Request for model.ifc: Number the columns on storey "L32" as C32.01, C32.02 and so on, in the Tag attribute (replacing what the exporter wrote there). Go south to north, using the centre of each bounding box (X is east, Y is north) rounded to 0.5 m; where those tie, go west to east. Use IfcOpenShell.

First a look at what the model holds.

```python
import ifcopenshell
import ifcopenshell.util.element
import ifcopenshell.util.placement

model = ifcopenshell.open("model.ifc")
print(model.schema)
storey = next(s for s in model.by_type("IfcBuildingStorey") if s.Name == "L32")
columns = [e for e in ifcopenshell.util.element.get_decomposition(storey) if e.is_a("IfcColumn")]
for e in sorted(columns, key=lambda e: e.id()):
    origin = ifcopenshell.util.placement.get_local_placement(e.ObjectPlacement)[:3, 3]
    print(e.id(), e.Tag, e.Name, origin.round(2) + 0.0, sep=" | ")
```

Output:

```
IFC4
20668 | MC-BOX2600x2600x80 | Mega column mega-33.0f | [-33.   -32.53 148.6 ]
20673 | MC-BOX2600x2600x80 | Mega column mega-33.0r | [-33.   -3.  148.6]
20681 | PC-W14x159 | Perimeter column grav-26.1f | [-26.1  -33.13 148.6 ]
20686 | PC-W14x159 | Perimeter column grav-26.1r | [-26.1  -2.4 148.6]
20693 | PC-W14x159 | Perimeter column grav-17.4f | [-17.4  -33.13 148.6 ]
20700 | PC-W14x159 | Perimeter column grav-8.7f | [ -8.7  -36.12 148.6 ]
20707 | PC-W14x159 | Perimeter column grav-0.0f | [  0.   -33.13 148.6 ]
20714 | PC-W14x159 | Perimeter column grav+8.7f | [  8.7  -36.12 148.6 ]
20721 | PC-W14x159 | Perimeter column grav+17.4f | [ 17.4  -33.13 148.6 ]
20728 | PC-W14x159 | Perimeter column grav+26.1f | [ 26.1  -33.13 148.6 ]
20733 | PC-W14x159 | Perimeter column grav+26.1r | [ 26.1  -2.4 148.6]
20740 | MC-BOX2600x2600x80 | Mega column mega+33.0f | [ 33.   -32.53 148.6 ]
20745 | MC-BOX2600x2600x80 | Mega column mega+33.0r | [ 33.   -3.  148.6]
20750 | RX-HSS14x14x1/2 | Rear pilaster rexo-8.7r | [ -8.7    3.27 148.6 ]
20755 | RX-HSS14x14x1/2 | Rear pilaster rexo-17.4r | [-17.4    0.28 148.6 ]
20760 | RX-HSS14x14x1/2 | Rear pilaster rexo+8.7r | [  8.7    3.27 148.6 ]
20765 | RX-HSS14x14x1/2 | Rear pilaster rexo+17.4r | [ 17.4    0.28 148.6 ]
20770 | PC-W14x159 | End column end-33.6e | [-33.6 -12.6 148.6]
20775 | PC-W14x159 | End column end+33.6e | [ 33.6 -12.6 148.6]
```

```python
import ifcopenshell
import ifcopenshell.geom
import ifcopenshell.util.element
import ifcopenshell.util.shape

model = ifcopenshell.open("model.ifc")
settings = ifcopenshell.geom.settings()
settings.set("use-world-coords", True)


def centre(element):
    shape = ifcopenshell.geom.create_shape(settings, element)
    return ifcopenshell.util.shape.get_bbox_centroid(shape.geometry)


storey = next(s for s in model.by_type("IfcBuildingStorey") if s.Name == "L32")
columns = [e for e in ifcopenshell.util.element.get_decomposition(storey) if e.is_a("IfcColumn")]

# Insertion points can sit at a corner or the storey origin, so sort by the geometry (in metres).
centres = {e: centre(e) for e in columns}
columns.sort(key=lambda e: (round(centres[e][1] / 0.5), centres[e][0]))

for i, e in enumerate(columns, start=1):
    number = f"C32.{i:02d}"
    e.Tag = number
    print(e.id(), number)

model.write("model_updated.ifc")
```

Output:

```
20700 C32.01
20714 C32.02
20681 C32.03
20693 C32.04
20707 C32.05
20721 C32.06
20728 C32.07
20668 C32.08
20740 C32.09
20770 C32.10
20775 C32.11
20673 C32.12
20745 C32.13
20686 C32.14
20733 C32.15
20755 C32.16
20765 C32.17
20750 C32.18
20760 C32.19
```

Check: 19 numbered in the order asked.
